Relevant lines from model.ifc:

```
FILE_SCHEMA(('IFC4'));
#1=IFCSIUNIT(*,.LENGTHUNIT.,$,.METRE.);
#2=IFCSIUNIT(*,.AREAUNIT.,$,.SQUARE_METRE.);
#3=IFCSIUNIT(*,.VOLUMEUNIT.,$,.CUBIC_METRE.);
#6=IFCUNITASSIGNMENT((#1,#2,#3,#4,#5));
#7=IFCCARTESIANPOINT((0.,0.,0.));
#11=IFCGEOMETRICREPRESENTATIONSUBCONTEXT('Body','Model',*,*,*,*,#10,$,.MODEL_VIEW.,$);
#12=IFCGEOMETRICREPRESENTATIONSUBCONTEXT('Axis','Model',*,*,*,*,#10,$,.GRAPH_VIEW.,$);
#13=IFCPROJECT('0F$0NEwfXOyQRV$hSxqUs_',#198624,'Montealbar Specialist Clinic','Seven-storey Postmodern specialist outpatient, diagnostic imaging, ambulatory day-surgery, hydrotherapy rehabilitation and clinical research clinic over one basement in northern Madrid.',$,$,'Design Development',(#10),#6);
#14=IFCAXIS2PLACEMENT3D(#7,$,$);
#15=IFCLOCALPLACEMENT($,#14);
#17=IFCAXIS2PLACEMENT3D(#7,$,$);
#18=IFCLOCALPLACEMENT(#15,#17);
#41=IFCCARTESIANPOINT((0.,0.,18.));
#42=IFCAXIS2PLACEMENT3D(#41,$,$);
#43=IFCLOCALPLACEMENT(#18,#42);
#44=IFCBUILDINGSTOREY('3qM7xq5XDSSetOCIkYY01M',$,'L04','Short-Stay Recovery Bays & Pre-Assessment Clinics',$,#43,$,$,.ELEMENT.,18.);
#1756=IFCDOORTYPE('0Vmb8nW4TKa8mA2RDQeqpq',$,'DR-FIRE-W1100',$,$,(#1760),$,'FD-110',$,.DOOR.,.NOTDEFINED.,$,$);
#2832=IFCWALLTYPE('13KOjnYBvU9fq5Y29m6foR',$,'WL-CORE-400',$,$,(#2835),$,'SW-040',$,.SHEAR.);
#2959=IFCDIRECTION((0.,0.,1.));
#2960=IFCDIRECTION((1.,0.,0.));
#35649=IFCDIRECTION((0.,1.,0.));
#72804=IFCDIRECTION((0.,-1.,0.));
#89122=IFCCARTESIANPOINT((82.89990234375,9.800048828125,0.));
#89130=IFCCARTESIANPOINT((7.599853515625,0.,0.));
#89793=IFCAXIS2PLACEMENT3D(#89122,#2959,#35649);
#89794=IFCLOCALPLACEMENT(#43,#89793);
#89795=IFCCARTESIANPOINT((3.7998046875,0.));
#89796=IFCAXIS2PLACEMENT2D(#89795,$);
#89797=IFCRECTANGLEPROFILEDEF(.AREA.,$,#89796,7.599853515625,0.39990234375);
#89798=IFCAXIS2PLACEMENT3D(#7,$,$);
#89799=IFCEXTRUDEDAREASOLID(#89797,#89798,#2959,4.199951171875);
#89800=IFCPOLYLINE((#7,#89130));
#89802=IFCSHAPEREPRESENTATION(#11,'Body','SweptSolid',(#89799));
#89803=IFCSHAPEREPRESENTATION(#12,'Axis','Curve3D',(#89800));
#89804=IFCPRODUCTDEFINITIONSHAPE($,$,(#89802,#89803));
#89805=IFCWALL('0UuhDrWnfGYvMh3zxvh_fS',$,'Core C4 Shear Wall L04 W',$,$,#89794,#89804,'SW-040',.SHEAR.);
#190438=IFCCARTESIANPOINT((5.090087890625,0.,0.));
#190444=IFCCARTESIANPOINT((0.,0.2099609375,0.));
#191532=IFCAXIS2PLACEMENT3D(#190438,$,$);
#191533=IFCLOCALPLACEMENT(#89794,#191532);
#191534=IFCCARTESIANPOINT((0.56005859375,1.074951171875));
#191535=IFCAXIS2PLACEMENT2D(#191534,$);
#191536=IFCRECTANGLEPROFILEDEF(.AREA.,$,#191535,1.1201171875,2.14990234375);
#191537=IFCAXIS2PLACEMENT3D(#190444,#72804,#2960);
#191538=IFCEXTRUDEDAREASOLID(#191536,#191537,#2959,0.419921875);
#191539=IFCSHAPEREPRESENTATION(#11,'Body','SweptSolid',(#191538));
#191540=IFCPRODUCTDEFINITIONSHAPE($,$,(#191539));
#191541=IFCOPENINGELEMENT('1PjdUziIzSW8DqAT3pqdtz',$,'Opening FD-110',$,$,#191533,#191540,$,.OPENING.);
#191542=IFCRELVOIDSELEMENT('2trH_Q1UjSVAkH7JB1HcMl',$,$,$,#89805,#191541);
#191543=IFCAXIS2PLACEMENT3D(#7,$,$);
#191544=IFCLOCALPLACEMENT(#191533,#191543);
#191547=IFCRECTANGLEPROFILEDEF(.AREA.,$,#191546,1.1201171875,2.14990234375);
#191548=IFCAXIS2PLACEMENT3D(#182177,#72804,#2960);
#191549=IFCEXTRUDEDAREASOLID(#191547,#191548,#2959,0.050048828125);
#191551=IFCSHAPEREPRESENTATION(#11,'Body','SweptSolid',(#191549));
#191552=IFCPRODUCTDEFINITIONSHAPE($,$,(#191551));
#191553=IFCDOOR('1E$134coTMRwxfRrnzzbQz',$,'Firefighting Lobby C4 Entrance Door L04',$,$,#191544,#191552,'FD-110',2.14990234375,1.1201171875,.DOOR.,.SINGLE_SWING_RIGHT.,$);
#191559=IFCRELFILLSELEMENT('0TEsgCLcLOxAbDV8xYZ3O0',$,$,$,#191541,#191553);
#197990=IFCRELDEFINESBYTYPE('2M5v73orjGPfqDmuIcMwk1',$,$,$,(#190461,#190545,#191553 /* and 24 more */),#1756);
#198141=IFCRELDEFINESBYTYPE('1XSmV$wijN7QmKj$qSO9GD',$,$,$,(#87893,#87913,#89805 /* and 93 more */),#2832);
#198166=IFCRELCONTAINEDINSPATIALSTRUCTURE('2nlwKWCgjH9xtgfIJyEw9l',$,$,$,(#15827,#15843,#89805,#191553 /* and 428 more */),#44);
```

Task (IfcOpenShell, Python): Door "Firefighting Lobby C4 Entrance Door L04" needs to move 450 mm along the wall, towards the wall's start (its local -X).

```python
import ifcopenshell
import ifcopenshell.api.geometry
import ifcopenshell.util.placement

model = ifcopenshell.open("model.ifc")

door = model.by_id(191553)
opening = door.FillsVoids[0].RelatingOpeningElement
wall = opening.VoidsElements[0].RelatingBuildingElement

wall_matrix = ifcopenshell.util.placement.get_local_placement(wall.ObjectPlacement)
shift = wall_matrix[:3, 0] * -0.45
before = ifcopenshell.util.placement.get_local_placement(door.ObjectPlacement)[:3, 3].copy()

# The door is placed relative to its opening, so it follows when the opening moves.
matrix = ifcopenshell.util.placement.get_local_placement(opening.ObjectPlacement)
matrix[:3, 3] += shift
ifcopenshell.api.geometry.edit_object_placement(
    model, product=opening, matrix=matrix, is_si=False, should_transform_children=True
)

after = ifcopenshell.util.placement.get_local_placement(door.ObjectPlacement)[:3, 3]
print("door moved by", (after - before).round(3) + 0.0)

model.write("model_edited.ifc")
```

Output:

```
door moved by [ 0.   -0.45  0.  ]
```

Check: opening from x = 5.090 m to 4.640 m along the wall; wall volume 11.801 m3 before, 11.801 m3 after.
